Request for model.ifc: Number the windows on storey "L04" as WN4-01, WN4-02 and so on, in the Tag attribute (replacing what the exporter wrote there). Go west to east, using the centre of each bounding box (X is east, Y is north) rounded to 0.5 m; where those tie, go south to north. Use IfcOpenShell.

First a look at what the model holds.

```python
import ifcopenshell
import ifcopenshell.util.element
import ifcopenshell.util.placement

model = ifcopenshell.open("model.ifc")
print(model.schema)
storey = next(s for s in model.by_type("IfcBuildingStorey") if s.Name == "L04")
windows = [e for e in ifcopenshell.util.element.get_decomposition(storey) if e.is_a("IfcWindow")]
for e in sorted(windows, key=lambda e: e.id()):
    origin = ifcopenshell.util.placement.get_local_placement(e.ObjectPlacement)[:3, 3]
    print(e.id(), e.Tag, e.Name, origin.round(2) + 0.0, sep=" | ")
```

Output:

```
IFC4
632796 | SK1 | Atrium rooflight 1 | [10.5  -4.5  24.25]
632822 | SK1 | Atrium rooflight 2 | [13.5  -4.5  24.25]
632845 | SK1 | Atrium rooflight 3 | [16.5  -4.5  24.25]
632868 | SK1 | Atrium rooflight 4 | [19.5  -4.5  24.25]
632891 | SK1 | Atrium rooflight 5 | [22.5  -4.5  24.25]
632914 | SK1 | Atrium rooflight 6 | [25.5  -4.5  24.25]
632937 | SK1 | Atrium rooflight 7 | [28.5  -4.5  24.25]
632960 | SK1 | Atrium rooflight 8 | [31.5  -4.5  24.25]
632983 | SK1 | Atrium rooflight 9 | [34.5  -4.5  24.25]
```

```python
import ifcopenshell
import ifcopenshell.geom
import ifcopenshell.util.element
import ifcopenshell.util.shape

model = ifcopenshell.open("model.ifc")
settings = ifcopenshell.geom.settings()
settings.set("use-world-coords", True)


def centre(element):
    shape = ifcopenshell.geom.create_shape(settings, element)
    return ifcopenshell.util.shape.get_bbox_centroid(shape.geometry)


storey = next(s for s in model.by_type("IfcBuildingStorey") if s.Name == "L04")
windows = [e for e in ifcopenshell.util.element.get_decomposition(storey) if e.is_a("IfcWindow")]

# Insertion points can sit at a corner or the storey origin, so sort by the geometry (in metres).
centres = {e: centre(e) for e in windows}
windows.sort(key=lambda e: (round(centres[e][0] / 0.5), centres[e][1]))

for i, e in enumerate(windows, start=1):
    number = f"WN4-{i:02d}"
    e.Tag = number
    print(e.id(), number)

model.write("model_edited.ifc")
```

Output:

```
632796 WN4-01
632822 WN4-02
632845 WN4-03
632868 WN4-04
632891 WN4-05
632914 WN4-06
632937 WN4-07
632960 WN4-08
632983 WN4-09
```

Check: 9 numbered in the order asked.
